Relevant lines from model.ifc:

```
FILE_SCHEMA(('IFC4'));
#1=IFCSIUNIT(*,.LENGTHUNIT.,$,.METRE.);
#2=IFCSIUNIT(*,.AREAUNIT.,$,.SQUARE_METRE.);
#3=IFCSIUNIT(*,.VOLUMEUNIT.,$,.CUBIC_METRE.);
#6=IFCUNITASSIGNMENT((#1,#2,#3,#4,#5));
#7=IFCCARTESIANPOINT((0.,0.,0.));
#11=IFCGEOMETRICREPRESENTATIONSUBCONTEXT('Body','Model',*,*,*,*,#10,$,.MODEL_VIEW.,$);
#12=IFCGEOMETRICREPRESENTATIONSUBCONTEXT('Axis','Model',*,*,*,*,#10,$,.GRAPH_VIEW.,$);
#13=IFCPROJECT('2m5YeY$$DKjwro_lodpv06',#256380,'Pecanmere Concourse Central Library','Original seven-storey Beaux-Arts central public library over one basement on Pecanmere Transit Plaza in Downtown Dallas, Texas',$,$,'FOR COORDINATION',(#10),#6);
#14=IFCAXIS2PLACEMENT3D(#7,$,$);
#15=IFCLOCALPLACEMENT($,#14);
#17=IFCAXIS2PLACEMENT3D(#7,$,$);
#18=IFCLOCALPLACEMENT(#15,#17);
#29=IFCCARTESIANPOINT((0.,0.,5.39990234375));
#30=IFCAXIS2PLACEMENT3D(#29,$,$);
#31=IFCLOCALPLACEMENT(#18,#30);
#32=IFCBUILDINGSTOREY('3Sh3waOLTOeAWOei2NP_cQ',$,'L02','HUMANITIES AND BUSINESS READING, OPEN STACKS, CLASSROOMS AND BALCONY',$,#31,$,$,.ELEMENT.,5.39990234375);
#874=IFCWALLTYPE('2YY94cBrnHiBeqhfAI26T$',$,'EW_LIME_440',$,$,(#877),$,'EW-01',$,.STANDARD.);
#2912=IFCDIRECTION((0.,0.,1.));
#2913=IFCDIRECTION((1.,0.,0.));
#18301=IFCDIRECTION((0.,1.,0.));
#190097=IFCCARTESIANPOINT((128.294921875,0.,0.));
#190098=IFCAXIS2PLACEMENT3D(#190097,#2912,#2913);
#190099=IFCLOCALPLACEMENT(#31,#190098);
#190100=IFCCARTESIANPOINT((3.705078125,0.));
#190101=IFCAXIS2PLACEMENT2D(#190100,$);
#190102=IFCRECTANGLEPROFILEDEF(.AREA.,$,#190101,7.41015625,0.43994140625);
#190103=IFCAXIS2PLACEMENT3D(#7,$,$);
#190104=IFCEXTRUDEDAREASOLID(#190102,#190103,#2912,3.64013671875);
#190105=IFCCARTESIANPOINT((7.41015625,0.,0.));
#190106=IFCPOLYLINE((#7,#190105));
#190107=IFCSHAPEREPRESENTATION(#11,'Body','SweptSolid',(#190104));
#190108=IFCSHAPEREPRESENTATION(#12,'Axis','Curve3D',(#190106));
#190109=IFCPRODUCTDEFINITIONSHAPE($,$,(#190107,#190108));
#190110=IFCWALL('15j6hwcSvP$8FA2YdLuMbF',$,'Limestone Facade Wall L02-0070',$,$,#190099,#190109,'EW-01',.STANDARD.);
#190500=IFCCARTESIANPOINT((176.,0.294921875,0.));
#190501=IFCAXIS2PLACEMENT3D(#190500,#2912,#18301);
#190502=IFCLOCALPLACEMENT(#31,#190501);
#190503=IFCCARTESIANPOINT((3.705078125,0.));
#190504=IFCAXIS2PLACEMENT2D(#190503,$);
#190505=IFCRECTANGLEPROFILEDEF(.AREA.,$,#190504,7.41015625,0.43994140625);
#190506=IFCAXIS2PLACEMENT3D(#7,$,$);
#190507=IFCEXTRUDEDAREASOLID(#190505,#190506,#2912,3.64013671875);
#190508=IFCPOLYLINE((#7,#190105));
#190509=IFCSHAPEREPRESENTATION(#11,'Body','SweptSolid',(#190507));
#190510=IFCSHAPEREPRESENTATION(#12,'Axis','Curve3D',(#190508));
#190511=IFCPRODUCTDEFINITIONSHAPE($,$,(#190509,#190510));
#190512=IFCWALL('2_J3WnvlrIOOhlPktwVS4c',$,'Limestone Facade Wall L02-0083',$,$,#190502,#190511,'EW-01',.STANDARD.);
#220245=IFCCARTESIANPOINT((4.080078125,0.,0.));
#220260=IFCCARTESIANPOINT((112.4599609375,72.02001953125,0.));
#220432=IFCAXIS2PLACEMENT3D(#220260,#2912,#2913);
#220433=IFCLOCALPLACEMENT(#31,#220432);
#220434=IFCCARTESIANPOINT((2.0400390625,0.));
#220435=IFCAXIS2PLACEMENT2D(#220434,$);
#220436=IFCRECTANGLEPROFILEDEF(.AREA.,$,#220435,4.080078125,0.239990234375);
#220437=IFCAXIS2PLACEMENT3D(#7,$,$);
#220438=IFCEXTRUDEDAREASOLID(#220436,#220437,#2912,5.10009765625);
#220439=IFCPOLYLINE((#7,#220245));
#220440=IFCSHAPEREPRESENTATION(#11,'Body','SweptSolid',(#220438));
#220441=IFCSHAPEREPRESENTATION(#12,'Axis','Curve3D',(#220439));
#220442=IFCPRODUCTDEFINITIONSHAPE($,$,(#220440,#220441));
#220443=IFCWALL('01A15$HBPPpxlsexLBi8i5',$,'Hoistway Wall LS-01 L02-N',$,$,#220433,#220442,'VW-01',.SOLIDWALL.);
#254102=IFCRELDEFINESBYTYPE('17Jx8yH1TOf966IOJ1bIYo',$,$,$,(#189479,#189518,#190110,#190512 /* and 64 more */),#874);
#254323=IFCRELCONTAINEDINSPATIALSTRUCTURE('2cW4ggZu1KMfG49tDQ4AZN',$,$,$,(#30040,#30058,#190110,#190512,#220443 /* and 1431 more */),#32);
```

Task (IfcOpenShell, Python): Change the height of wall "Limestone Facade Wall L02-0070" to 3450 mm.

```python
import ifcopenshell
import ifcopenshell.geom
import ifcopenshell.util.representation
import ifcopenshell.util.shape
import ifcopenshell.util.unit

model = ifcopenshell.open("model.ifc")
unit_scale = ifcopenshell.util.unit.calculate_unit_scale(model)
settings = ifcopenshell.geom.settings()


def volume(element):
    """Net volume in cubic metres, openings subtracted."""
    shape = ifcopenshell.geom.create_shape(settings, element)
    return ifcopenshell.util.shape.get_volume(shape.geometry)


wall = model.by_guid("15j6hwcSvP$8FA2YdLuMbF")
before = volume(wall)

body = ifcopenshell.util.representation.get_representation(wall, "Model", "Body")
solid = body.Items[0]
old_height = solid.Depth
solid.Depth = 3.45 / unit_scale
after = volume(wall)

print(f"height {old_height:g} -> {solid.Depth:g}, volume {before:.3f} -> {after:.3f} m3")

model.write("model-out.ifc")
```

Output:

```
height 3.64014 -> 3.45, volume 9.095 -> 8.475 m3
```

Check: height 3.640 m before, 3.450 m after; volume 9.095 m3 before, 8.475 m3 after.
